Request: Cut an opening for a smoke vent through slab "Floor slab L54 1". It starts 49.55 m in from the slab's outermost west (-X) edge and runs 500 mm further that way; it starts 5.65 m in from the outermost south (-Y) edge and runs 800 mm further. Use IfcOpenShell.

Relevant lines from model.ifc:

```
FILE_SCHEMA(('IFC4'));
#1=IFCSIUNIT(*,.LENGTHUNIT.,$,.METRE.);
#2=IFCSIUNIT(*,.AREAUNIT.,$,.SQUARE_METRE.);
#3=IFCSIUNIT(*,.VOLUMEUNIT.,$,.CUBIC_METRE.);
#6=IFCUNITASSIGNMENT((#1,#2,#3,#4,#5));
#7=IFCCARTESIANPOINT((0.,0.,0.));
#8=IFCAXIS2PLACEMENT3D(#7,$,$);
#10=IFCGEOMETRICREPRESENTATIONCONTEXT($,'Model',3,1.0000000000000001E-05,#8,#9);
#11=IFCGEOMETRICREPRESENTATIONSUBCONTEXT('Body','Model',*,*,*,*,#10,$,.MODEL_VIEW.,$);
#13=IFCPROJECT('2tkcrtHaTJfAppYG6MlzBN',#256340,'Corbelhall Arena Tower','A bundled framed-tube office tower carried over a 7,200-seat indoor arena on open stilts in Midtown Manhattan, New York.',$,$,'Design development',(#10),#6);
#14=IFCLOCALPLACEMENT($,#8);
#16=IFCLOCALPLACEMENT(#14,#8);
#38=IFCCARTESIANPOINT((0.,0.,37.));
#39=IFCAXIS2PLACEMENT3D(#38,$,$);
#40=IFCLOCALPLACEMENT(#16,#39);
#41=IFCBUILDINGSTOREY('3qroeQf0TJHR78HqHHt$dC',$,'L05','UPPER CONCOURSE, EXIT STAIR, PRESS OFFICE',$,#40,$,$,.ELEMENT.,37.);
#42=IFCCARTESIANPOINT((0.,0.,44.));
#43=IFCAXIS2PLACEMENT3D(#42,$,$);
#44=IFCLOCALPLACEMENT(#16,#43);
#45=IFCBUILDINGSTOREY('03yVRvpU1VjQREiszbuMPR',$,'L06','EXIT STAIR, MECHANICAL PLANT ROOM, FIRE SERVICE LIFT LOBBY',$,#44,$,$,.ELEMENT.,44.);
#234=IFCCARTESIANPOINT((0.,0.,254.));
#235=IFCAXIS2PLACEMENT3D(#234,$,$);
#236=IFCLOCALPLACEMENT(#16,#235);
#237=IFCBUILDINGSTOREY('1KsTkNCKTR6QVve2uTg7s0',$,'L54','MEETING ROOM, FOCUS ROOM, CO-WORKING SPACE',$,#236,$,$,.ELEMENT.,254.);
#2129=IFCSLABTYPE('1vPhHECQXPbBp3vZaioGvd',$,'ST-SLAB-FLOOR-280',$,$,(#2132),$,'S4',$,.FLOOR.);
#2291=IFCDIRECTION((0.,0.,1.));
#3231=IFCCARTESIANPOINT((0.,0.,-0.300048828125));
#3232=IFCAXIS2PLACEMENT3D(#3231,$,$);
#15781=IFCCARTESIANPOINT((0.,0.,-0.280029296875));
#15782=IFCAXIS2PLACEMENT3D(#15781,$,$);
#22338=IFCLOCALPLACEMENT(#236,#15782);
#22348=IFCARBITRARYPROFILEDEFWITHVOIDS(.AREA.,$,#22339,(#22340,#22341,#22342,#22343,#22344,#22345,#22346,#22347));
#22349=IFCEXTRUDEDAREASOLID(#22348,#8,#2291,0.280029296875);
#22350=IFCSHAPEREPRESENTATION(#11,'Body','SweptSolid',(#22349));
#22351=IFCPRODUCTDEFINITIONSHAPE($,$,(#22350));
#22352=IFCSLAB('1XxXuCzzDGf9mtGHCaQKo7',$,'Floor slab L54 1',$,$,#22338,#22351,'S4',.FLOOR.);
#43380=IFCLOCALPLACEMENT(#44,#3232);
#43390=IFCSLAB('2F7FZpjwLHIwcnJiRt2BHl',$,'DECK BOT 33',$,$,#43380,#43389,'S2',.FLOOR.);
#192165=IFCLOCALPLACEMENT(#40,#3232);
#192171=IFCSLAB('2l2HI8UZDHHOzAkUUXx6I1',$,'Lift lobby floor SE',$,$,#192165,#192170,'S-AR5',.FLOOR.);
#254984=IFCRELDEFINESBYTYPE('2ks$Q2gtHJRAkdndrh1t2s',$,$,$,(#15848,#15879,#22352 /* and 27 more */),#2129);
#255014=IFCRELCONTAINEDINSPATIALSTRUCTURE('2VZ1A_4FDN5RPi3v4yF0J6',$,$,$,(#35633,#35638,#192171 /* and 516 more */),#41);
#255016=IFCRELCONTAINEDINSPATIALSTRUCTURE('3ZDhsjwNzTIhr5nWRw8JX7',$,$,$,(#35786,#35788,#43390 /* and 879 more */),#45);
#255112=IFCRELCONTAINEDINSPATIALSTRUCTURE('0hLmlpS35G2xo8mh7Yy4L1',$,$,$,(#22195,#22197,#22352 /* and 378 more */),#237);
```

```python
import numpy as np
import ifcopenshell
import ifcopenshell.api.feature
import ifcopenshell.api.geometry
import ifcopenshell.api.root
import ifcopenshell.geom
import ifcopenshell.util.placement
import ifcopenshell.util.representation
import ifcopenshell.util.shape
import ifcopenshell.util.unit

model = ifcopenshell.open("model.ifc")
unit_scale = ifcopenshell.util.unit.calculate_unit_scale(model)
settings = ifcopenshell.geom.settings()


def volume(element):
    """Net volume in cubic metres, openings subtracted."""
    shape = ifcopenshell.geom.create_shape(settings, element)
    return ifcopenshell.util.shape.get_volume(shape.geometry)


slab = model.by_guid("1XxXuCzzDGf9mtGHCaQKo7")
before = volume(slab)

# Extent in the slab's own axes, in metres. The edges named are its -X and -Y sides.
slab_shape = ifcopenshell.geom.create_shape(settings, slab)
vertices = ifcopenshell.util.shape.get_vertices(slab_shape.geometry)
x_min, y_min, bottom = vertices.min(axis=0)
top = vertices[:, 2].max()

opening = ifcopenshell.api.root.create_entity(model, ifc_class="IfcOpeningElement", name="Smoke vent opening", predefined_type="OPENING")
context = ifcopenshell.util.representation.get_context(model, "Model", "Body", "MODEL_VIEW")
width, depth = 0.5, 0.8
outline = [(0.0, 0.0), (width, 0.0), (width, depth), (0.0, depth), (0.0, 0.0)]
# Overshoot both faces by 50 mm so the cut is clean.
shape = ifcopenshell.api.geometry.add_slab_representation(
    model, context=context, depth=top - bottom + 0.1, polyline=outline
)
ifcopenshell.api.geometry.assign_representation(model, product=opening, representation=shape)

matrix = ifcopenshell.util.placement.get_local_placement(slab.ObjectPlacement)
matrix[:, 3] = matrix @ np.append(np.array([x_min + 49.55, y_min + 5.65, bottom - 0.05]) / unit_scale, 1.0)
ifcopenshell.api.geometry.edit_object_placement(model, product=opening, matrix=matrix, is_si=False)
ifcopenshell.api.feature.add_feature(model, feature=opening, element=slab)

after = volume(slab)

print(f"slab volume {before:.3f} -> {after:.3f} m3")

model.write("model_rev.ifc")
```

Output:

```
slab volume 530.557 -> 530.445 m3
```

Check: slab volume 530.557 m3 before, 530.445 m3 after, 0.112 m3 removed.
